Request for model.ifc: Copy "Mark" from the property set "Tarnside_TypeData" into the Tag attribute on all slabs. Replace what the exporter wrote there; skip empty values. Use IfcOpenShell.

First a look at what the model holds.

```python
import ifcopenshell
import ifcopenshell.util.element

model = ifcopenshell.open("model.ifc")
print(model.schema)
slabs = model.by_type("IfcSlab")
print(len(slabs), "slabs")
for e in slabs[:8]:
    source = ifcopenshell.util.element.get_pset(e, "Tarnside_TypeData", "Mark")
    target = e.Tag
    print(e.id(), repr(source), repr(target), sep=" | ")
```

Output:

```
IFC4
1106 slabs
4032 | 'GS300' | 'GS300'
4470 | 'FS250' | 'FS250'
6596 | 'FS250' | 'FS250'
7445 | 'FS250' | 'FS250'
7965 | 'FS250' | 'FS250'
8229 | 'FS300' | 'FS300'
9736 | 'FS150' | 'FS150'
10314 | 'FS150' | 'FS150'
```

```python
import ifcopenshell
import ifcopenshell.util.element

model = ifcopenshell.open("model.ifc")

count = 0
for e in model.by_type("IfcSlab"):
    value = ifcopenshell.util.element.get_pset(e, "Tarnside_TypeData", "Mark")
    current = e.Tag
    if not value or not value.strip() or current == value:
        continue
    e.Tag = value
    count += 1

print(count, "slabs updated")

model.write("model_edited.ifc")
```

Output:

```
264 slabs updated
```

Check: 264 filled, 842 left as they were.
